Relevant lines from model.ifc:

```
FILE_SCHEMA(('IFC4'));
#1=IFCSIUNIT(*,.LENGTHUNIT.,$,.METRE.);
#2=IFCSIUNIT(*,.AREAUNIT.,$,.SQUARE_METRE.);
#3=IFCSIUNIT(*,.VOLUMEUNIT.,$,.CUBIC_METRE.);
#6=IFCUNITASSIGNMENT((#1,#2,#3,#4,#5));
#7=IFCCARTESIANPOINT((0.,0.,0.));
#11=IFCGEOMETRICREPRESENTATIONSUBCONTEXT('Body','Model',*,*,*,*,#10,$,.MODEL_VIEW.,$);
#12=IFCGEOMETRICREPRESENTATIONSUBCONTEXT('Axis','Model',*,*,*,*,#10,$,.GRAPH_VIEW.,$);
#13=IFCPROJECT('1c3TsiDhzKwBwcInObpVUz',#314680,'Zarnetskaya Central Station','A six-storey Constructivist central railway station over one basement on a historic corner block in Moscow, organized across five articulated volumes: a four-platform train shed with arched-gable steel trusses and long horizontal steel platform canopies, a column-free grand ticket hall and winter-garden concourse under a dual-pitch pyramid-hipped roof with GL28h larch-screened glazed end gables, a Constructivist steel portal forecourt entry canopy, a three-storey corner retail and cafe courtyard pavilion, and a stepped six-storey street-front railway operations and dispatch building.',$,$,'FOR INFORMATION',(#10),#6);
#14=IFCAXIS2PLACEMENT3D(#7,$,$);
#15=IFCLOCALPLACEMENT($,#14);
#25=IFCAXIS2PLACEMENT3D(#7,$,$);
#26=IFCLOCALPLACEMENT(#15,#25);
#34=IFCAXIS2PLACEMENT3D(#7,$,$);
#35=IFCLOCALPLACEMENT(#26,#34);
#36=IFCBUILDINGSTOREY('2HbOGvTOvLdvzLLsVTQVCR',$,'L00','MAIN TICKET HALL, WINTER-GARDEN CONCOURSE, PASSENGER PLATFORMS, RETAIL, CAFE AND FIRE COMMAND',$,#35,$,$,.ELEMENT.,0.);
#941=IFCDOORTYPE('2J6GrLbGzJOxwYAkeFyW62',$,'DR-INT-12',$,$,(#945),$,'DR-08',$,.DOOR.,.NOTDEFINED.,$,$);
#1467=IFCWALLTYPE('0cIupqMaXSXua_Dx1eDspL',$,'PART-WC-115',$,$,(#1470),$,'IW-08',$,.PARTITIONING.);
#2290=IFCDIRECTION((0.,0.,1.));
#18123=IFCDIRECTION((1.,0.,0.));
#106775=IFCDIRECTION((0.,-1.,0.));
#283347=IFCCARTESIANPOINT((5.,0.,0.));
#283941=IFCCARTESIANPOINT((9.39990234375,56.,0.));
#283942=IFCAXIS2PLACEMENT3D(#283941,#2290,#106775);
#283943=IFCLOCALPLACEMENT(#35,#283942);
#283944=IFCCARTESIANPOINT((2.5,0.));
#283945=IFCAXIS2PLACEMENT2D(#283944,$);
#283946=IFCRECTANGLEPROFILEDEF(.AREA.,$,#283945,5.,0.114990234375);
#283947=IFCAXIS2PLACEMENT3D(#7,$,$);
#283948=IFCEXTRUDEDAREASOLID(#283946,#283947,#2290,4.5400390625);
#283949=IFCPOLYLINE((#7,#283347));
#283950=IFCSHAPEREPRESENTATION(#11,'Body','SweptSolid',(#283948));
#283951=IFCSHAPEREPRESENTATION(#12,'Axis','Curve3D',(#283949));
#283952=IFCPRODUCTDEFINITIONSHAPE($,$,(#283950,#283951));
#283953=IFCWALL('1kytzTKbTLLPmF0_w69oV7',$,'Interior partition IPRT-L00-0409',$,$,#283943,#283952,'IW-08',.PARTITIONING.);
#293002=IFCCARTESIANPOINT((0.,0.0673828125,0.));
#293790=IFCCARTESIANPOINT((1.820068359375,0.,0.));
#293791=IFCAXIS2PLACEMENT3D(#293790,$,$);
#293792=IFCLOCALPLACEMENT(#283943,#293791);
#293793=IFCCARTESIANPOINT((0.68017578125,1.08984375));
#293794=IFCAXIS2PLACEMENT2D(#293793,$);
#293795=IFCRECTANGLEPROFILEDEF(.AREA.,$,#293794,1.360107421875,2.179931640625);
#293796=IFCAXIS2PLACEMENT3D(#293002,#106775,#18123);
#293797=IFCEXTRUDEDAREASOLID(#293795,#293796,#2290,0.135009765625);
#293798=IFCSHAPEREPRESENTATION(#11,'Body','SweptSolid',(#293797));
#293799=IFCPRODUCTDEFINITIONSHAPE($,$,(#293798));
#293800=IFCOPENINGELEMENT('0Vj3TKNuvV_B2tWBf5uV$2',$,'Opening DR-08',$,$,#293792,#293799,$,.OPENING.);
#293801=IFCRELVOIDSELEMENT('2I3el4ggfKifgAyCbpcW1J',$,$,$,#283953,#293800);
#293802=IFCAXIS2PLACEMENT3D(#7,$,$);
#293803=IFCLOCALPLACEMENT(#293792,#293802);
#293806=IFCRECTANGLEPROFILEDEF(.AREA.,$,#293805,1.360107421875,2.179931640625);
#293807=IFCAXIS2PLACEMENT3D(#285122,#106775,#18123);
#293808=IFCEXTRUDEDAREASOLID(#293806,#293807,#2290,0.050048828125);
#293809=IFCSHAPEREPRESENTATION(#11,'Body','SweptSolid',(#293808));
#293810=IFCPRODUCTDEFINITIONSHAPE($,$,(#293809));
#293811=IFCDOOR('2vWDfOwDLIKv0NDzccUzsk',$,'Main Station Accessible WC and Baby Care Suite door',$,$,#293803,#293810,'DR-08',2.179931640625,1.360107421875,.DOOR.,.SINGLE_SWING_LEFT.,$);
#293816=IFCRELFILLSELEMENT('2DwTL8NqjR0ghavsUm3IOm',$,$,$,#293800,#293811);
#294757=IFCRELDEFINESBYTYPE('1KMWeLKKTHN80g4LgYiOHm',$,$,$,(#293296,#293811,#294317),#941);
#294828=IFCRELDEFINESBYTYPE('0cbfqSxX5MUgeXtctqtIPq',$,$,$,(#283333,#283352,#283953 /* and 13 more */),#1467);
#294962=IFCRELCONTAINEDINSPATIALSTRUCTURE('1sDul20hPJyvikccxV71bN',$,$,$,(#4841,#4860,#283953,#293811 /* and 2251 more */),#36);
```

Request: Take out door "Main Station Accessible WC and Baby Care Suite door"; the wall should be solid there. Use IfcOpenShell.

```python
import ifcopenshell
import ifcopenshell.api.feature
import ifcopenshell.api.root
import ifcopenshell.geom
import ifcopenshell.util.shape

model = ifcopenshell.open("model.ifc")
settings = ifcopenshell.geom.settings()


def volume(element):
    """Net volume in cubic metres, openings subtracted."""
    shape = ifcopenshell.geom.create_shape(settings, element)
    return ifcopenshell.util.shape.get_volume(shape.geometry)


door = model.by_id(293811)
opening = door.FillsVoids[0].RelatingOpeningElement
wall = opening.VoidsElements[0].RelatingBuildingElement
before = volume(wall)

ifcopenshell.api.root.remove_product(model, product=door)
ifcopenshell.api.feature.remove_feature(model, feature=opening)

after = volume(wall)

print(f"wall volume {before:.3f} -> {after:.3f} m3")

model.write("model_v2.ifc")
```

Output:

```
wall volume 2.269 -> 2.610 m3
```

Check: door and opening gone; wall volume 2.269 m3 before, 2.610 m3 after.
